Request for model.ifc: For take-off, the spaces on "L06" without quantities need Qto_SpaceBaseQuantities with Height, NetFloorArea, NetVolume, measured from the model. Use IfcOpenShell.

First a look at what the model holds.

```python
import ifcopenshell
import ifcopenshell.util.element
import ifcopenshell.util.unit

model = ifcopenshell.open("model.ifc")
print(model.schema)
for unit_type in ("LENGTHUNIT", "AREAUNIT", "VOLUMEUNIT"):
    print(unit_type, ifcopenshell.util.unit.calculate_unit_scale(model, unit_type))
storey = next(s for s in model.by_type("IfcBuildingStorey") if s.Name == "L06")
spaces = [e for e in ifcopenshell.util.element.get_decomposition(storey) if e.is_a("IfcSpace")]
for e in sorted(spaces, key=lambda e: e.id()):
    print(e.id(), e.is_a(), e.Name, list(ifcopenshell.util.element.get_psets(e, qtos_only=True)), sep=" | ")
```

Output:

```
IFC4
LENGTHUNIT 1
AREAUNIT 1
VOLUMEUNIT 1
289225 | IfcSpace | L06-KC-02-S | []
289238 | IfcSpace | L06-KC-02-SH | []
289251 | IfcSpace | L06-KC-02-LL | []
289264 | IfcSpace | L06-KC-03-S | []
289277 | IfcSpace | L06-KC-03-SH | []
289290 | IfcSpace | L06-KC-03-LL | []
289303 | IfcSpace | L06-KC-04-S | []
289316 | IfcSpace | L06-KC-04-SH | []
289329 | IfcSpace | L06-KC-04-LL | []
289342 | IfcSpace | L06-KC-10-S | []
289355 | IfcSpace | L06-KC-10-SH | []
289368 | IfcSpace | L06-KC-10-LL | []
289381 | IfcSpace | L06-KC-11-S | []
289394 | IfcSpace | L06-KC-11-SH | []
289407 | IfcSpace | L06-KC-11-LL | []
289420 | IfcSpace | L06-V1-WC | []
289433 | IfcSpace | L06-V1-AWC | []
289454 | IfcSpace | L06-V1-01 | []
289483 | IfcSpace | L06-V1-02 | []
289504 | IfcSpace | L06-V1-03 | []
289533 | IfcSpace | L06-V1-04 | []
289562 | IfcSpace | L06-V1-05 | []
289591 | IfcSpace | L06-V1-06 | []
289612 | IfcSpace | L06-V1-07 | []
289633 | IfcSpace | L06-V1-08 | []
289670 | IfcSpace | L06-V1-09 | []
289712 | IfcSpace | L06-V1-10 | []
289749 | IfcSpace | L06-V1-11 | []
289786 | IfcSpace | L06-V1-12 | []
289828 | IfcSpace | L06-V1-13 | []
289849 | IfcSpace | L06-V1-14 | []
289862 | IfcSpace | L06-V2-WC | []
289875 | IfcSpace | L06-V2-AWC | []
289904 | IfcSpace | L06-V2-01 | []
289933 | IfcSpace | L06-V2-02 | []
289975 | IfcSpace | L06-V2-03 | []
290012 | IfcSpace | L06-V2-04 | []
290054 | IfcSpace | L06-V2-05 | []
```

```python
import ifcopenshell
import ifcopenshell.api.pset
import ifcopenshell.geom
import ifcopenshell.util.element
import ifcopenshell.util.shape
import ifcopenshell.util.unit

model = ifcopenshell.open("model.ifc")
unit_scale = ifcopenshell.util.unit.calculate_unit_scale(model)
area_scale = ifcopenshell.util.unit.calculate_unit_scale(model, "AREAUNIT")
volume_scale = ifcopenshell.util.unit.calculate_unit_scale(model, "VOLUMEUNIT")
settings = ifcopenshell.geom.settings()

storey = next(s for s in model.by_type("IfcBuildingStorey") if s.Name == "L06")
spaces = [e for e in ifcopenshell.util.element.get_decomposition(storey) if e.is_a("IfcSpace")]

for e in sorted(spaces, key=lambda e: e.id()):
    if ifcopenshell.util.element.get_psets(e, qtos_only=True, should_inherit=False):
        continue
    # Geometry comes back in metres, in the element's own axes.
    shape = ifcopenshell.geom.create_shape(settings, e)
    values = {
        "Height": ifcopenshell.util.shape.get_z(shape.geometry) / unit_scale,
        "NetFloorArea": ifcopenshell.util.shape.get_footprint_area(shape.geometry) / area_scale,
        "NetVolume": ifcopenshell.util.shape.get_volume(shape.geometry) / volume_scale,
    }
    qto = ifcopenshell.api.pset.add_qto(model, product=e, name="Qto_SpaceBaseQuantities")
    ifcopenshell.api.pset.edit_qto(model, qto=qto, properties=values)
    print(e.id(), {k: round(v, 3) for k, v in values.items()})

model.write("model_rev.ifc")
```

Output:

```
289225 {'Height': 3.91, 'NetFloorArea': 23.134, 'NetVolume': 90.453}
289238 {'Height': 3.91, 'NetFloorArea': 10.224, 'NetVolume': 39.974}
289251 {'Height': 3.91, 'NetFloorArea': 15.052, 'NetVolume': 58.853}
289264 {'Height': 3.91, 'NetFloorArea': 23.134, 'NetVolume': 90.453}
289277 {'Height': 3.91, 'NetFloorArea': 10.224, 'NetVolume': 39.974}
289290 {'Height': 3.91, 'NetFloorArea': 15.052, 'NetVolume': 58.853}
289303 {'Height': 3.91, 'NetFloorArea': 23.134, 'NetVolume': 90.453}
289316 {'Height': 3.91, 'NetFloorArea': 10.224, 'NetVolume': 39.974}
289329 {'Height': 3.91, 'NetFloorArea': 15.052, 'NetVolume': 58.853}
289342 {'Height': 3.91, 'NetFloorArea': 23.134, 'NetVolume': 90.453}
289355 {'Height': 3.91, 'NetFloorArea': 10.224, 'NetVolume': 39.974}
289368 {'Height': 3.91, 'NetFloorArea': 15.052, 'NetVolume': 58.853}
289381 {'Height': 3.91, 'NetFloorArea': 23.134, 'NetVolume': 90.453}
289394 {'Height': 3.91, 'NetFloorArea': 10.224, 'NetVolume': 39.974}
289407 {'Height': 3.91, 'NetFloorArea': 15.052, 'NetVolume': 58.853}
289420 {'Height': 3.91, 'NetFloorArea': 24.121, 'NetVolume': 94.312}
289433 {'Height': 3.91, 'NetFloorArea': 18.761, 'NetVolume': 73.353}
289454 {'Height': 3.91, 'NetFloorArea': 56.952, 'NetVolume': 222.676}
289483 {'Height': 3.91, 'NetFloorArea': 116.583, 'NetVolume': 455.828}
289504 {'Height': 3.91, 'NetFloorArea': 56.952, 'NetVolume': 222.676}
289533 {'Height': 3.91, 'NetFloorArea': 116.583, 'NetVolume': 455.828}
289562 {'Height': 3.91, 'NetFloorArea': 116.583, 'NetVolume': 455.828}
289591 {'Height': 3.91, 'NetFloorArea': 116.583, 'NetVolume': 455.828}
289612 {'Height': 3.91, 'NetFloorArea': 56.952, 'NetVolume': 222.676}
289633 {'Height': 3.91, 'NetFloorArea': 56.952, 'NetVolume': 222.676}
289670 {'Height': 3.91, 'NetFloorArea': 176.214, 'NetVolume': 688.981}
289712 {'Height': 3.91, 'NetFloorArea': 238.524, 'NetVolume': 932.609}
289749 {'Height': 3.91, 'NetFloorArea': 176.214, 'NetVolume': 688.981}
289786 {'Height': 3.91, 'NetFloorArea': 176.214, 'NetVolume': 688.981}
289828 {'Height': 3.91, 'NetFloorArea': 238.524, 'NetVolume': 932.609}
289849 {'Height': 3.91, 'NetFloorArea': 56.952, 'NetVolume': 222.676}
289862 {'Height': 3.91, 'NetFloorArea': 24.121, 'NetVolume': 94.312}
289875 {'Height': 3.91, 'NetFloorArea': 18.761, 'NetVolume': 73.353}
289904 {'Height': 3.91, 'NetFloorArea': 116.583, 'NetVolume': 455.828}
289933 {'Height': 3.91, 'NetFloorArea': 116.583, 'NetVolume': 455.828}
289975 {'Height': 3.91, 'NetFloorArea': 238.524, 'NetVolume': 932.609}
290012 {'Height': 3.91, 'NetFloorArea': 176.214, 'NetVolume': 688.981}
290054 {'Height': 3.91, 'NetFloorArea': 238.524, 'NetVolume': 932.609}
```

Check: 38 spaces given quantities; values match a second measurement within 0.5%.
